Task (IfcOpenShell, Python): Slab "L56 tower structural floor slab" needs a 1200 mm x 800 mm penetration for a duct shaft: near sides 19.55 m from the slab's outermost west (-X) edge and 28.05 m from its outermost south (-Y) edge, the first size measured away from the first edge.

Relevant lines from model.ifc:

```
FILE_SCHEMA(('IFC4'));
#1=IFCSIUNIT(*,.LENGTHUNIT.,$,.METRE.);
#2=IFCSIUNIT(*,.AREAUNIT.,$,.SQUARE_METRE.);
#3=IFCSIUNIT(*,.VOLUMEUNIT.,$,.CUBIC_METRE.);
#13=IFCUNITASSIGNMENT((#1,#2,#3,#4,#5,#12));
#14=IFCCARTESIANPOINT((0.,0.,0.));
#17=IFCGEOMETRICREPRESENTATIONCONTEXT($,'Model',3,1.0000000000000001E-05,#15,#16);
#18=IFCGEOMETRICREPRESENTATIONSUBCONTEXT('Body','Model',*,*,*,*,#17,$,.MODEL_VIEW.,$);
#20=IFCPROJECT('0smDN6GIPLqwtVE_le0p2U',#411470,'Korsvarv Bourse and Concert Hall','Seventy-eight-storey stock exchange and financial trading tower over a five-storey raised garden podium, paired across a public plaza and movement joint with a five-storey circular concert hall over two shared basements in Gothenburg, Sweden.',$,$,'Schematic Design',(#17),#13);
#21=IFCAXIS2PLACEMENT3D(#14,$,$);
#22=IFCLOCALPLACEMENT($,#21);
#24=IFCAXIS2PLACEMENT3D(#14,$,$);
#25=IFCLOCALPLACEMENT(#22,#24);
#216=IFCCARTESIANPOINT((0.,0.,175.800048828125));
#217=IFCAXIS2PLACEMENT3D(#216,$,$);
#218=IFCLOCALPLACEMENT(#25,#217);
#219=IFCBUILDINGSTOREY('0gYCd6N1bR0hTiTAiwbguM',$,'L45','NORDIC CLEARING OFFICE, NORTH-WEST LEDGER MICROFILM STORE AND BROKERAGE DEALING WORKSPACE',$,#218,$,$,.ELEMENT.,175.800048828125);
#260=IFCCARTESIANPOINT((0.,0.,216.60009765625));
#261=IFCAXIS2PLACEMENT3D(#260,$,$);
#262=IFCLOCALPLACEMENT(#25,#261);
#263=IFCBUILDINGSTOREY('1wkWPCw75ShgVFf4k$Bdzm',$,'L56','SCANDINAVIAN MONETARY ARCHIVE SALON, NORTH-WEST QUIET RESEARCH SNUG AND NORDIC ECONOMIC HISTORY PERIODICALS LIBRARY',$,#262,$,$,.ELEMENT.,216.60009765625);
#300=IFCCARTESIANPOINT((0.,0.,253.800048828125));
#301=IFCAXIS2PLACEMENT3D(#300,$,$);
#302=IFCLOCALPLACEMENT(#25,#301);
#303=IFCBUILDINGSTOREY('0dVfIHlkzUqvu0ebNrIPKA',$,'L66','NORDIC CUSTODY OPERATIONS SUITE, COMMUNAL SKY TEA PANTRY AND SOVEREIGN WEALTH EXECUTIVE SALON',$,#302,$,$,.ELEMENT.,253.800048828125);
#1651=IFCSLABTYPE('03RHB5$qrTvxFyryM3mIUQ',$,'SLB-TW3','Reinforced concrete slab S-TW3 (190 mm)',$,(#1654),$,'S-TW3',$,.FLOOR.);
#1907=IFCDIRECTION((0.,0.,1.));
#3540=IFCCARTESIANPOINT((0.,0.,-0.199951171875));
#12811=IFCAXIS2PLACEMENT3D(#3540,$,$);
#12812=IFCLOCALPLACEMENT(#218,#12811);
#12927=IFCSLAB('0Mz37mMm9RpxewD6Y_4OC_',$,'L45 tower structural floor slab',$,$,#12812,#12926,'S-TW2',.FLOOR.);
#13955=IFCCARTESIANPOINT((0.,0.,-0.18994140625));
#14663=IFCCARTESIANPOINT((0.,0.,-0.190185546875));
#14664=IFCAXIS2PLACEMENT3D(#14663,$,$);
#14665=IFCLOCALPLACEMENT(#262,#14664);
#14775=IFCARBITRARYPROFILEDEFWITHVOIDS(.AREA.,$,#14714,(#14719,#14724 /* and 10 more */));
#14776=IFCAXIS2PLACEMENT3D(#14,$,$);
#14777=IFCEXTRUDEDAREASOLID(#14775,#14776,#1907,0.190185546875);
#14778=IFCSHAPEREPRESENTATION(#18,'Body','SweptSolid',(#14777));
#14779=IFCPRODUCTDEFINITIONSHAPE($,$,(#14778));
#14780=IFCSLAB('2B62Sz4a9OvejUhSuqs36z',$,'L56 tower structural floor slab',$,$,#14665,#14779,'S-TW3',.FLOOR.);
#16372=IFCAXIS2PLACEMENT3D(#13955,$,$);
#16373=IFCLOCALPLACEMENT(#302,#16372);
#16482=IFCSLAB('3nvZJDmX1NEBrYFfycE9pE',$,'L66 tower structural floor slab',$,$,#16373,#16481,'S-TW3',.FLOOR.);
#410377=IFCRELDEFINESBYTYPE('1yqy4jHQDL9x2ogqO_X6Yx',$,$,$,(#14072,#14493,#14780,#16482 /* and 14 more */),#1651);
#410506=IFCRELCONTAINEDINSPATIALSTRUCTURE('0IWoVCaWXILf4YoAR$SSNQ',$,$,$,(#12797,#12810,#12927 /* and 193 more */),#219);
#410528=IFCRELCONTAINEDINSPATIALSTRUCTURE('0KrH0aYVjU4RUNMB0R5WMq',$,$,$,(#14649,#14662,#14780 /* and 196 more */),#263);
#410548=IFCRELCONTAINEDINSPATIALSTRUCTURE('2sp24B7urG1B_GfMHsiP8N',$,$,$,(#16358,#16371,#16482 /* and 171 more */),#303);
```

```python
import numpy as np
import ifcopenshell
import ifcopenshell.api.feature
import ifcopenshell.api.geometry
import ifcopenshell.api.root
import ifcopenshell.geom
import ifcopenshell.util.placement
import ifcopenshell.util.representation
import ifcopenshell.util.shape
import ifcopenshell.util.unit

model = ifcopenshell.open("model.ifc")
unit_scale = ifcopenshell.util.unit.calculate_unit_scale(model)
settings = ifcopenshell.geom.settings()


def volume(element):
    """Net volume in cubic metres, openings subtracted."""
    shape = ifcopenshell.geom.create_shape(settings, element)
    return ifcopenshell.util.shape.get_volume(shape.geometry)


slab = model.by_guid("2B62Sz4a9OvejUhSuqs36z")
before = volume(slab)

# Extent in the slab's own axes, in metres. The edges named are its -X and -Y sides.
slab_shape = ifcopenshell.geom.create_shape(settings, slab)
vertices = ifcopenshell.util.shape.get_vertices(slab_shape.geometry)
x_min, y_min, bottom = vertices.min(axis=0)
top = vertices[:, 2].max()

opening = ifcopenshell.api.root.create_entity(model, ifc_class="IfcOpeningElement", name="Duct shaft opening", predefined_type="OPENING")
context = ifcopenshell.util.representation.get_context(model, "Model", "Body", "MODEL_VIEW")
width, depth = 1.2, 0.8
outline = [(0.0, 0.0), (width, 0.0), (width, depth), (0.0, depth), (0.0, 0.0)]
# Overshoot both faces by 50 mm so the cut is clean.
shape = ifcopenshell.api.geometry.add_slab_representation(
    model, context=context, depth=top - bottom + 0.1, polyline=outline
)
ifcopenshell.api.geometry.assign_representation(model, product=opening, representation=shape)

matrix = ifcopenshell.util.placement.get_local_placement(slab.ObjectPlacement)
matrix[:, 3] = matrix @ np.append(np.array([x_min + 19.55, y_min + 28.05, bottom - 0.05]) / unit_scale, 1.0)
ifcopenshell.api.geometry.edit_object_placement(model, product=opening, matrix=matrix, is_si=False)
ifcopenshell.api.feature.add_feature(model, feature=opening, element=slab)

after = volume(slab)

print(f"slab volume {before:.3f} -> {after:.3f} m3")

model.write("model_updated.ifc")
```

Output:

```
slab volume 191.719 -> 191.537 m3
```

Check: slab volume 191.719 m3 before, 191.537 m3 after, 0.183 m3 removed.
